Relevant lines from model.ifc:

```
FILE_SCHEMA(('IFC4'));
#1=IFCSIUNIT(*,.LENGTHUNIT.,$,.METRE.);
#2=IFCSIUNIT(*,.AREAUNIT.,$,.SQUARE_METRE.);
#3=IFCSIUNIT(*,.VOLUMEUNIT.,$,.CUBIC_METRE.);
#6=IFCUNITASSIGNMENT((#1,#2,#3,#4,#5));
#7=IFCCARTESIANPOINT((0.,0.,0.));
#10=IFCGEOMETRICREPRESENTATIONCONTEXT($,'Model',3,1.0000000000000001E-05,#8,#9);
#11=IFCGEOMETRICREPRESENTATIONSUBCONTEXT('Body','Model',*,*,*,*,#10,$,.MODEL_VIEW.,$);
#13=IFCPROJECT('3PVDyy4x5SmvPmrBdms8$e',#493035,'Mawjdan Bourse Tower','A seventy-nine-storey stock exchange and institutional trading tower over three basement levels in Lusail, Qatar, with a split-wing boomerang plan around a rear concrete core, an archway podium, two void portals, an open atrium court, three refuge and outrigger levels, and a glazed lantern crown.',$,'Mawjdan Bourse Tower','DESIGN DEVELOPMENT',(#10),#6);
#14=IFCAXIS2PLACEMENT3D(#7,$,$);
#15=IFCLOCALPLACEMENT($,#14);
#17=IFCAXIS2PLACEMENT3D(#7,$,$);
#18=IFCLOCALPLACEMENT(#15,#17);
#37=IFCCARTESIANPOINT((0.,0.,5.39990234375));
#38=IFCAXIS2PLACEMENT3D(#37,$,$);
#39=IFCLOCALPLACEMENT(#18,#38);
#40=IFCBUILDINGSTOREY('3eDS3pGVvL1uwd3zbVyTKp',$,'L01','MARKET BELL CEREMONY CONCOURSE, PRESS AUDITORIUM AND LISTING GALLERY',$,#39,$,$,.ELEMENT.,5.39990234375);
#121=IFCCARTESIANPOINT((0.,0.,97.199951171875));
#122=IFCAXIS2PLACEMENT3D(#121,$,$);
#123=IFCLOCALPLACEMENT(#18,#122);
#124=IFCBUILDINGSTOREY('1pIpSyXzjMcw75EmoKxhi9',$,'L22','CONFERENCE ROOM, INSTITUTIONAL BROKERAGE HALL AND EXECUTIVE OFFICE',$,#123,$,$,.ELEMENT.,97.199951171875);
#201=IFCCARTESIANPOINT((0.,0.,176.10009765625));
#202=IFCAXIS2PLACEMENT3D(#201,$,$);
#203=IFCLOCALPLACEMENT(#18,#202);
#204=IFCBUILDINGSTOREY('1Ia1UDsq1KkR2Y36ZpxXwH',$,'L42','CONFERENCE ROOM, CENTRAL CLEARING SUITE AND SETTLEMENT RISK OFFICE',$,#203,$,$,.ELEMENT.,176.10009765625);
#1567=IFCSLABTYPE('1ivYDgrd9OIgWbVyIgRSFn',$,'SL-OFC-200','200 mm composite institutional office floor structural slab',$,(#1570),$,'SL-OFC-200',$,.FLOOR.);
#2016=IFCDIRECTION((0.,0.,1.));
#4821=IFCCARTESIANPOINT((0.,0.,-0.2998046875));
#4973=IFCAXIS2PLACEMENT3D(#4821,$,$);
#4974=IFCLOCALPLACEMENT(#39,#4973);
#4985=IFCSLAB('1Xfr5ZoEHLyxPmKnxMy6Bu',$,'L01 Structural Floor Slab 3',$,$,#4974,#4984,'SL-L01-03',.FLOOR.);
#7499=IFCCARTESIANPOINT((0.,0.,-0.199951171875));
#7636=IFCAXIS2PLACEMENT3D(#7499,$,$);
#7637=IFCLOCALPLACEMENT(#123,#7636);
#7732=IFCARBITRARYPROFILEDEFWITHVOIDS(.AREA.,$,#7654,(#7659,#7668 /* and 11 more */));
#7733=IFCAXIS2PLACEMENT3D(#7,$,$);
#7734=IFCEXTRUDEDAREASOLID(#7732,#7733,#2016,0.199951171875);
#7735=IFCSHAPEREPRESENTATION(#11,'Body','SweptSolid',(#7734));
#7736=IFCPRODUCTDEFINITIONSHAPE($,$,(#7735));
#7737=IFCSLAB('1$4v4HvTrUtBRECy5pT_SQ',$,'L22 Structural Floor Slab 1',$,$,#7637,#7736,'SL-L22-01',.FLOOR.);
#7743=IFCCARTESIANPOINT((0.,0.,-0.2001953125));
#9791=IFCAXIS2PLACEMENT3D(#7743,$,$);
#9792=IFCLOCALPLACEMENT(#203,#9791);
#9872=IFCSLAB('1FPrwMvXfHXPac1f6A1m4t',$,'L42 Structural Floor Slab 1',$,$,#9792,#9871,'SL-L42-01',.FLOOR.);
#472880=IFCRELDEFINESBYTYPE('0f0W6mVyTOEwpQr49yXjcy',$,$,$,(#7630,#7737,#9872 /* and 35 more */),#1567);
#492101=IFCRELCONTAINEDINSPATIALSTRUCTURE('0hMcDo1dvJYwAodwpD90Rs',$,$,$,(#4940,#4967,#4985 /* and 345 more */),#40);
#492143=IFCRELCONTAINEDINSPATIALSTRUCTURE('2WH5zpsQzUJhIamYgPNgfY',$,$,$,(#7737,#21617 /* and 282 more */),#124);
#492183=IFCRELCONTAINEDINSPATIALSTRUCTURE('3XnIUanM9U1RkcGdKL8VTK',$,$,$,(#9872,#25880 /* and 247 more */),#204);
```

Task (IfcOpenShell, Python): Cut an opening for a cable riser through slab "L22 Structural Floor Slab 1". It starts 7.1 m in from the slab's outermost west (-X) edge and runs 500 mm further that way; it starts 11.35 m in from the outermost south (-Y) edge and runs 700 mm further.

```python
import numpy as np
import ifcopenshell
import ifcopenshell.api.feature
import ifcopenshell.api.geometry
import ifcopenshell.api.root
import ifcopenshell.geom
import ifcopenshell.util.placement
import ifcopenshell.util.representation
import ifcopenshell.util.shape
import ifcopenshell.util.unit

model = ifcopenshell.open("model.ifc")
unit_scale = ifcopenshell.util.unit.calculate_unit_scale(model)
settings = ifcopenshell.geom.settings()


def volume(element):
    """Net volume in cubic metres, openings subtracted."""
    shape = ifcopenshell.geom.create_shape(settings, element)
    return ifcopenshell.util.shape.get_volume(shape.geometry)


slab = model.by_id(7737)
before = volume(slab)

# Extent in the slab's own axes, in metres. The edges named are its -X and -Y sides.
slab_shape = ifcopenshell.geom.create_shape(settings, slab)
vertices = ifcopenshell.util.shape.get_vertices(slab_shape.geometry)
x_min, y_min, bottom = vertices.min(axis=0)
top = vertices[:, 2].max()

opening = ifcopenshell.api.root.create_entity(model, ifc_class="IfcOpeningElement", name="Cable riser opening", predefined_type="OPENING")
context = ifcopenshell.util.representation.get_context(model, "Model", "Body", "MODEL_VIEW")
width, depth = 0.5, 0.7
outline = [(0.0, 0.0), (width, 0.0), (width, depth), (0.0, depth), (0.0, 0.0)]
# Overshoot both faces by 50 mm so the cut is clean.
shape = ifcopenshell.api.geometry.add_slab_representation(
    model, context=context, depth=top - bottom + 0.1, polyline=outline
)
ifcopenshell.api.geometry.assign_representation(model, product=opening, representation=shape)

matrix = ifcopenshell.util.placement.get_local_placement(slab.ObjectPlacement)
matrix[:, 3] = matrix @ np.append(np.array([x_min + 7.1, y_min + 11.35, bottom - 0.05]) / unit_scale, 1.0)
ifcopenshell.api.geometry.edit_object_placement(model, product=opening, matrix=matrix, is_si=False)
ifcopenshell.api.feature.add_feature(model, feature=opening, element=slab)

after = volume(slab)

print(f"slab volume {before:.3f} -> {after:.3f} m3")

model.write("model-out.ifc")
```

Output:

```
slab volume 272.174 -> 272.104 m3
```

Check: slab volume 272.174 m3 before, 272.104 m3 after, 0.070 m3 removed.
